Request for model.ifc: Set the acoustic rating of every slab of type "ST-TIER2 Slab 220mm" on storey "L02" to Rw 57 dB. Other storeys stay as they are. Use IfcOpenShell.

First a look at what the model holds.

```python
import ifcopenshell
import ifcopenshell.util.element

model = ifcopenshell.open("model.ifc")
print(model.schema)
storey = next(s for s in model.by_type("IfcBuildingStorey") if s.Name == "L02")
slabs = [e for e in ifcopenshell.util.element.get_decomposition(storey) if e.is_a("IfcSlab")]
seen = {}
for e in slabs:
    element_type = ifcopenshell.util.element.get_type(e)
    key = (element_type.Name if element_type != e and element_type else None, ifcopenshell.util.element.get_pset(e, "Pset_SlabCommon", "AcousticRating"))
    seen[key] = seen.get(key, 0) + 1
for (name, value), count in sorted(seen.items(), key=str):
    print(count, "x", name, "|", value)
```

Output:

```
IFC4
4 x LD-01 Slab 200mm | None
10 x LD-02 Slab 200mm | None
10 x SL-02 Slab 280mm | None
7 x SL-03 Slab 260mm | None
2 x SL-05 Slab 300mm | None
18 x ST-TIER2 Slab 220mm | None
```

```python
import ifcopenshell
import ifcopenshell.api.pset
import ifcopenshell.util.element

model = ifcopenshell.open("model.ifc")

storey = next(s for s in model.by_type("IfcBuildingStorey") if s.Name == "L02")
slabs = [e for e in ifcopenshell.util.element.get_decomposition(storey) if e.is_a("IfcSlab")]

count = 0
for e in slabs:
    element_type = ifcopenshell.util.element.get_type(e)
    if element_type in (None, e) or element_type.Name != "ST-TIER2 Slab 220mm":
        continue
    # add_pset returns the element's existing set when there is one.
    pset = ifcopenshell.api.pset.add_pset(model, product=e, name="Pset_SlabCommon")
    ifcopenshell.api.pset.edit_pset(model, pset=pset, properties={"AcousticRating": "Rw 57 dB"})
    count += 1

print(count, "slabs updated")

model.write("model_updated.ifc")
```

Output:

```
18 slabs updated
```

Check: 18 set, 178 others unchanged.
